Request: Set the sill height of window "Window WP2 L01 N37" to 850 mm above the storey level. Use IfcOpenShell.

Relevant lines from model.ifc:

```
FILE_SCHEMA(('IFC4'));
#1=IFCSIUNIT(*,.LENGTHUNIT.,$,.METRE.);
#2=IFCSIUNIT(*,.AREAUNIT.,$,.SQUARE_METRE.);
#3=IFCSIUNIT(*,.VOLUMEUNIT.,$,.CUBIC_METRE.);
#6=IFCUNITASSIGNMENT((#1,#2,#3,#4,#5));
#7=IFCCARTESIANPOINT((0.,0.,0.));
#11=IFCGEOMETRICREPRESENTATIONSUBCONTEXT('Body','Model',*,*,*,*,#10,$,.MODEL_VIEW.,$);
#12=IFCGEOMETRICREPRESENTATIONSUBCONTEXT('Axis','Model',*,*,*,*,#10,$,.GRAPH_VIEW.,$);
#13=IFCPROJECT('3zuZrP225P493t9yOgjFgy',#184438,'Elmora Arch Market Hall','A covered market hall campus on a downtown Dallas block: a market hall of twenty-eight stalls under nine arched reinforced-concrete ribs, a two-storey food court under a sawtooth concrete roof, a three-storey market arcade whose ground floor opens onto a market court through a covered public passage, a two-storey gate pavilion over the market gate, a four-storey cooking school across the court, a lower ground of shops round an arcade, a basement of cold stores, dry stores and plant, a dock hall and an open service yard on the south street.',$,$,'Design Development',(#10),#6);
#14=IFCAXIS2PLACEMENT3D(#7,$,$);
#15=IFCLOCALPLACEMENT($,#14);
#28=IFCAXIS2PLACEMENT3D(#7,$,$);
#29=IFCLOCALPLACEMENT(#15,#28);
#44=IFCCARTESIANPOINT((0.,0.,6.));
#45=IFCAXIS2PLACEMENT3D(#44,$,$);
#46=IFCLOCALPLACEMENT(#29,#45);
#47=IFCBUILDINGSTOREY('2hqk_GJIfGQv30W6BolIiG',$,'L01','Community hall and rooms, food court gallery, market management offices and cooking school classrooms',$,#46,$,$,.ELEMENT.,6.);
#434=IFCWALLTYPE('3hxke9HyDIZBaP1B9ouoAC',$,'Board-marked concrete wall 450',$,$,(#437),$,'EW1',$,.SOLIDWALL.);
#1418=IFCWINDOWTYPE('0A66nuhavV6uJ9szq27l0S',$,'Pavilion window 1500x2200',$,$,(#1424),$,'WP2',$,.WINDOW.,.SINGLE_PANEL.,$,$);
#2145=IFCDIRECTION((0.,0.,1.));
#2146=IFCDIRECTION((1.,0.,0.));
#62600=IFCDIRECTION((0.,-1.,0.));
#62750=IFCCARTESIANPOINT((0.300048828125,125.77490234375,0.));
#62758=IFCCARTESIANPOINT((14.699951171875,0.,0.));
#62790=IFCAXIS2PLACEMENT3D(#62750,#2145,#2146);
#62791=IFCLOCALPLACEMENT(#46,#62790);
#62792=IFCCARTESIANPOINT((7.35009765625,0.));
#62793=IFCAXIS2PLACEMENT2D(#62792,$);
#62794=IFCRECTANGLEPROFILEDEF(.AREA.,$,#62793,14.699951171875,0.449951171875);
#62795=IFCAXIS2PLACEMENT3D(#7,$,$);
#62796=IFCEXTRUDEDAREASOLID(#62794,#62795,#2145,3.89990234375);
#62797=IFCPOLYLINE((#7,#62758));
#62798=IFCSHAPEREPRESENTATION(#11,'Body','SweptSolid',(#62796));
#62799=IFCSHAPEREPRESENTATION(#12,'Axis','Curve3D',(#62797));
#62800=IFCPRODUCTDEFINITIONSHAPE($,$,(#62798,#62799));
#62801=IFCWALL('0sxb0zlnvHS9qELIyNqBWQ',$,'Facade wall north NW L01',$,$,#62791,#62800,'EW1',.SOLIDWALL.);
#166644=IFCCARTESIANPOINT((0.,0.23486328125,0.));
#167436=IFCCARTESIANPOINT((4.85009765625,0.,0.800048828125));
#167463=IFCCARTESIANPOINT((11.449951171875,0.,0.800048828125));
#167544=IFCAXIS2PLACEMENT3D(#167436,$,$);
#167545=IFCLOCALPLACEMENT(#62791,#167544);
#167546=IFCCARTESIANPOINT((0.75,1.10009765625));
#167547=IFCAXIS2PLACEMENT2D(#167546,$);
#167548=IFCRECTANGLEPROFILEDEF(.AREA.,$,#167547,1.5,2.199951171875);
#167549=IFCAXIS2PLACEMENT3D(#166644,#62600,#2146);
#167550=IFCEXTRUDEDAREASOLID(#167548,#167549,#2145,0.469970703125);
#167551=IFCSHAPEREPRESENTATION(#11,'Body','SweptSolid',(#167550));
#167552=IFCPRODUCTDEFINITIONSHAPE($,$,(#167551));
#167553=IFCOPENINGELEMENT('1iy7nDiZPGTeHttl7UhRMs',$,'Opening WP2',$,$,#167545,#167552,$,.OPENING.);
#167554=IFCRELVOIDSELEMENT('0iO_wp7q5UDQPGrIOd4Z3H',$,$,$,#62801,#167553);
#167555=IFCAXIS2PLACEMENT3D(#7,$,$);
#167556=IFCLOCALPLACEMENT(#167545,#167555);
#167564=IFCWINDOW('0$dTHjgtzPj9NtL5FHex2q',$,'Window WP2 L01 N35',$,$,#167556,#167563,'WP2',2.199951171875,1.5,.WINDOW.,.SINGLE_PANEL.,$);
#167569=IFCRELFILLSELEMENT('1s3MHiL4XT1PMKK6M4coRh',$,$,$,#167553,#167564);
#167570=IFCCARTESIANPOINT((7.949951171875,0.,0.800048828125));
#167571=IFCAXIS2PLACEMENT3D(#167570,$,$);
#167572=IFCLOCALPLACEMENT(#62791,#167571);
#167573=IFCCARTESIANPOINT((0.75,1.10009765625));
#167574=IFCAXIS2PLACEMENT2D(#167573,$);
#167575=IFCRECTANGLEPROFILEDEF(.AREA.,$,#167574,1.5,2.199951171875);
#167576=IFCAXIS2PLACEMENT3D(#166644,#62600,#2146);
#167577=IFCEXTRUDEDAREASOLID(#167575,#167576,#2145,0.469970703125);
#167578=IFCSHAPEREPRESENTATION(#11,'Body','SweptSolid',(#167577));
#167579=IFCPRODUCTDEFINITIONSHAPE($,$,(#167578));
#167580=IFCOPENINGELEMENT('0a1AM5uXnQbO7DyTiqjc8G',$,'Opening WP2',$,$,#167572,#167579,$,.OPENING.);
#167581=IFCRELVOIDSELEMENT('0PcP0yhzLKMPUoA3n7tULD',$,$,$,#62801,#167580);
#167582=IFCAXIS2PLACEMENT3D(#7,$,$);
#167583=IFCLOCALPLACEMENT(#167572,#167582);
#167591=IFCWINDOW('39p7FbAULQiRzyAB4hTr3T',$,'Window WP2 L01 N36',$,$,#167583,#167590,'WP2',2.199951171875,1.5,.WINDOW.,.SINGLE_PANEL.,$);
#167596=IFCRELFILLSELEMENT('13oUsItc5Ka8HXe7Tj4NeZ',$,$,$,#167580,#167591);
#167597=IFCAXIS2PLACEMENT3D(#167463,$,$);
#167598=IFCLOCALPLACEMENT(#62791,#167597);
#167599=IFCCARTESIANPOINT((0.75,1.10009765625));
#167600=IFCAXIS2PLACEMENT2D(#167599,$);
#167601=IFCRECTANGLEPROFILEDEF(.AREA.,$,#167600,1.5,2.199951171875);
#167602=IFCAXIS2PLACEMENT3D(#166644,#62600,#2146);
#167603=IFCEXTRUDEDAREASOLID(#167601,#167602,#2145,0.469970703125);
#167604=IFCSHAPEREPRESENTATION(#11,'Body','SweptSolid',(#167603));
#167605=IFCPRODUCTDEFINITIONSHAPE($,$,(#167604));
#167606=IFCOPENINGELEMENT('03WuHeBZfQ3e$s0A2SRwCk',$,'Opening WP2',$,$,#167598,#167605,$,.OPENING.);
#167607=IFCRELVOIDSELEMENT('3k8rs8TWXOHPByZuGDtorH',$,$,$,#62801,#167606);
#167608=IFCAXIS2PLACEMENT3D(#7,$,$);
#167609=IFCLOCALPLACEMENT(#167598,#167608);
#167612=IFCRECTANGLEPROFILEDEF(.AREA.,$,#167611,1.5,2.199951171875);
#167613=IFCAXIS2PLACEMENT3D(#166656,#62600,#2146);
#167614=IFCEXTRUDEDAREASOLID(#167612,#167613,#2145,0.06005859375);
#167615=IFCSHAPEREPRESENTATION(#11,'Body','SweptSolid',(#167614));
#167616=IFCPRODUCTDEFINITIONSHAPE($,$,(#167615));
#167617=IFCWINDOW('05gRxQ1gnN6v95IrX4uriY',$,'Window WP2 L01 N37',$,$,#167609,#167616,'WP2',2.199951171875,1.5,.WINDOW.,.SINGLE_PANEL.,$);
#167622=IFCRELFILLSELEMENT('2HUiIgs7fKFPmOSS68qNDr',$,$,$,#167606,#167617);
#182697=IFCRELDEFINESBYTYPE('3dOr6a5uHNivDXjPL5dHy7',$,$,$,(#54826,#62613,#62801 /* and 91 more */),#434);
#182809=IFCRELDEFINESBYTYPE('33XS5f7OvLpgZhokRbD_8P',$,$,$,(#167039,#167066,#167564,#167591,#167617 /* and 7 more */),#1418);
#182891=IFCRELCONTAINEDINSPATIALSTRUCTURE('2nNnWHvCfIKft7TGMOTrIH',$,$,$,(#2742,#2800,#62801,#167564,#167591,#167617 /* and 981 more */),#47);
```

```python
import numpy as np
import ifcopenshell
import ifcopenshell.api.geometry
import ifcopenshell.geom
import ifcopenshell.util.element
import ifcopenshell.util.placement
import ifcopenshell.util.shape
import ifcopenshell.util.unit

model = ifcopenshell.open("model.ifc")
unit_scale = ifcopenshell.util.unit.calculate_unit_scale(model)

window = model.by_guid("05gRxQ1gnN6v95IrX4uriY")
opening = window.FillsVoids[0].RelatingOpeningElement
storey = ifcopenshell.util.element.get_container(window, ifc_class="IfcBuildingStorey")
level = ifcopenshell.util.placement.get_local_placement(storey.ObjectPlacement)[2, 3]

# The opening's origin need not be at the sill, so measure its lowest point.
shape = ifcopenshell.geom.create_shape(ifcopenshell.geom.settings(), opening)
bottom = ifcopenshell.util.shape.get_shape_bottom_elevation(shape, shape.geometry) / unit_scale
dz = level + 0.85 / unit_scale - bottom

shift = np.array([0.0, 0.0, dz])
# The window is placed relative to its opening, so it follows when the opening moves.
matrix = ifcopenshell.util.placement.get_local_placement(opening.ObjectPlacement)
matrix[:3, 3] += shift
ifcopenshell.api.geometry.edit_object_placement(
    model, product=opening, matrix=matrix, is_si=False, should_transform_children=True
)

print(f"moved by {dz * unit_scale:+.3f} m")

model.write("model_updated.ifc")
```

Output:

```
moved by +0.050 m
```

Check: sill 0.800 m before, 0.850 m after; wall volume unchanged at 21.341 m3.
